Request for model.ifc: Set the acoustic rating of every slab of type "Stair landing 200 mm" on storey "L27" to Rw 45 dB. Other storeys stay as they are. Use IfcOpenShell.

First a look at what the model holds.

```python
import ifcopenshell
import ifcopenshell.util.element

model = ifcopenshell.open("model.ifc")
print(model.schema)
storey = next(s for s in model.by_type("IfcBuildingStorey") if s.Name == "L27")
slabs = [e for e in ifcopenshell.util.element.get_decomposition(storey) if e.is_a("IfcSlab")]
seen = {}
for e in slabs:
    element_type = ifcopenshell.util.element.get_type(e)
    key = (element_type.Name if element_type != e and element_type else None, ifcopenshell.util.element.get_pset(e, "Pset_SlabCommon", "AcousticRating"))
    seen[key] = seen.get(key, 0) + 1
for (name, value), count in sorted(seen.items(), key=str):
    print(count, "x", name, "|", value)
```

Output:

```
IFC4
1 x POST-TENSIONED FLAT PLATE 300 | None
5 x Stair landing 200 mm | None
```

```python
import ifcopenshell
import ifcopenshell.api.pset
import ifcopenshell.util.element

model = ifcopenshell.open("model.ifc")

storey = next(s for s in model.by_type("IfcBuildingStorey") if s.Name == "L27")
slabs = [e for e in ifcopenshell.util.element.get_decomposition(storey) if e.is_a("IfcSlab")]

count = 0
for e in slabs:
    element_type = ifcopenshell.util.element.get_type(e)
    if element_type in (None, e) or element_type.Name != "Stair landing 200 mm":
        continue
    found = ifcopenshell.util.element.get_pset(e, "Pset_SlabCommon", should_inherit=False)
    if found:
        pset = model.by_id(found["id"])
        if len(ifcopenshell.util.element.get_elements_by_pset(pset)) > 1:
            pset = ifcopenshell.api.pset.unshare_pset(model, products=[e], pset=pset)[0]
    else:
        pset = ifcopenshell.api.pset.add_pset(model, product=e, name="Pset_SlabCommon")
    ifcopenshell.api.pset.edit_pset(model, pset=pset, properties={"AcousticRating": "Rw 45 dB"})
    count += 1

print(count, "slabs updated")

model.write("model_rev.ifc")
```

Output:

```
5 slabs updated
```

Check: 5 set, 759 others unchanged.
